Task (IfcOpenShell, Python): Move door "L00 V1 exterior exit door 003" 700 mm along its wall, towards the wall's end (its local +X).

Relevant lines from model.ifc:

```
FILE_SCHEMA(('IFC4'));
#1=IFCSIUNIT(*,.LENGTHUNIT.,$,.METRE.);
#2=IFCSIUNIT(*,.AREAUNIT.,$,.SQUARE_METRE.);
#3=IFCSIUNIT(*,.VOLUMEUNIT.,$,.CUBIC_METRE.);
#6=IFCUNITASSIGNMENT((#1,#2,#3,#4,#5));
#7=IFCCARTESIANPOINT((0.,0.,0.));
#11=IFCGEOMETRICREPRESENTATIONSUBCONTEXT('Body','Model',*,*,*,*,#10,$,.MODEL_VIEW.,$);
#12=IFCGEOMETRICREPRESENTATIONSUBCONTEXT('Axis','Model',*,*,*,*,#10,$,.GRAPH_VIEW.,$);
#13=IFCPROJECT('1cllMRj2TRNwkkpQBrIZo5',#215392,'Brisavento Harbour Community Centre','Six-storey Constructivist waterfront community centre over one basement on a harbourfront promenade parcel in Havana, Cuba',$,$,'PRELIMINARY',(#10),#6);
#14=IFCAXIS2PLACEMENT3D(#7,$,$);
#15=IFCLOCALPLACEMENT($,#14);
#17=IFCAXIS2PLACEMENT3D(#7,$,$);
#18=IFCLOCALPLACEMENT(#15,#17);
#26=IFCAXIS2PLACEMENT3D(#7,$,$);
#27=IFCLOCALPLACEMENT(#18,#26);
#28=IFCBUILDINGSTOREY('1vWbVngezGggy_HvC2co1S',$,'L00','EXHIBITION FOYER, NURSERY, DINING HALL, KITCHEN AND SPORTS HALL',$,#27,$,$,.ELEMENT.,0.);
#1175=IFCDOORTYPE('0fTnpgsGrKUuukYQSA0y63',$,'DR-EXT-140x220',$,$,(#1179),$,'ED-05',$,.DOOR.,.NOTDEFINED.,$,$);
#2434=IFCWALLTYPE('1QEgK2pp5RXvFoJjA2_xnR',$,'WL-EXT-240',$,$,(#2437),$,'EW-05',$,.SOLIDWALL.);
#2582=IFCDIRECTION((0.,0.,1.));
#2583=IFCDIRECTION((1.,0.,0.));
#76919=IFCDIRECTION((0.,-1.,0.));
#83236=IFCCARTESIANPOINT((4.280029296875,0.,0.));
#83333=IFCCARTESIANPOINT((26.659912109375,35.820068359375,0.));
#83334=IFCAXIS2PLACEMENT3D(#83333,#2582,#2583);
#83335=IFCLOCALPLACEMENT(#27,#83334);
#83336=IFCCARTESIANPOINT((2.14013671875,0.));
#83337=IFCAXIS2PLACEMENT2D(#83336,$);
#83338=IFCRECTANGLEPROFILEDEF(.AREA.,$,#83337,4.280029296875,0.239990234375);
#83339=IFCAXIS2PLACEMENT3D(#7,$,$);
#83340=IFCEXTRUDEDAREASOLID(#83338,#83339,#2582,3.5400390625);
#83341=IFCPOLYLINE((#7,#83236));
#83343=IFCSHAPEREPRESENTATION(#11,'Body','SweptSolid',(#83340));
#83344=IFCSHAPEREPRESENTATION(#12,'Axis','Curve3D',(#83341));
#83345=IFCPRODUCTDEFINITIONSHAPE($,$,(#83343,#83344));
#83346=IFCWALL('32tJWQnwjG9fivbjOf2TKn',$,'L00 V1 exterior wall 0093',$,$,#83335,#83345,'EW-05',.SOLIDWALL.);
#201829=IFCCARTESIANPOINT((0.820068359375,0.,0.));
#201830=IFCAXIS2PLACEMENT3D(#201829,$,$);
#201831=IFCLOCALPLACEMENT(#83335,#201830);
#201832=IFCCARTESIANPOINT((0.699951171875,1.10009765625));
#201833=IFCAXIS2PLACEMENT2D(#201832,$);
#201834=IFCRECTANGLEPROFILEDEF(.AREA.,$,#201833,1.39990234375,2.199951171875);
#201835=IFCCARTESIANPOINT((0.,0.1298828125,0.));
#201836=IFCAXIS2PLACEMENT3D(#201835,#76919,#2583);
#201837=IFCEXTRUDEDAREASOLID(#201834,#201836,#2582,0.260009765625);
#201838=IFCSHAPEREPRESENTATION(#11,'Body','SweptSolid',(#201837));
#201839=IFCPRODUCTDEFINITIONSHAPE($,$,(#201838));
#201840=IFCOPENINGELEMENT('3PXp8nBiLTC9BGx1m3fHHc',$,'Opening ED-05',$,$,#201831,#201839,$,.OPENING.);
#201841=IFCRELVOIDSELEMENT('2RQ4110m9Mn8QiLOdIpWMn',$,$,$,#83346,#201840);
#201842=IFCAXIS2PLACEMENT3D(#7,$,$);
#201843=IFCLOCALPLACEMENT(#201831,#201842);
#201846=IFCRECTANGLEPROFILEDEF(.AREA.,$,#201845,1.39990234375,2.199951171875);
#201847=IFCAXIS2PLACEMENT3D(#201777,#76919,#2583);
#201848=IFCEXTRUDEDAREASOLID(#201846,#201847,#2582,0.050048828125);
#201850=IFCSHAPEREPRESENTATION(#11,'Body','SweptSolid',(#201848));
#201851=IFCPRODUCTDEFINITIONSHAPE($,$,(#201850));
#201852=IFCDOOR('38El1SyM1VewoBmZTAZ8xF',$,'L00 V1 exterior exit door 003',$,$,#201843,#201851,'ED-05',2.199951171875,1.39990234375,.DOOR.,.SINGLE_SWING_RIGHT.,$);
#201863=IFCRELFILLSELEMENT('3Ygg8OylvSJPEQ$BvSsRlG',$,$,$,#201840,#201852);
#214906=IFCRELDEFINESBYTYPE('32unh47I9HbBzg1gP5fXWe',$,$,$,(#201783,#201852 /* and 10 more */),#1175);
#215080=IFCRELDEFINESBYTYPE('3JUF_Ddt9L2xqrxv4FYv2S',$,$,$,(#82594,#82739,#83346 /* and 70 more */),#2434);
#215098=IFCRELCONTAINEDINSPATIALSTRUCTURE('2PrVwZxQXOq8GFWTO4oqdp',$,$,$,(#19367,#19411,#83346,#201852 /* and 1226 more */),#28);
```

```python
import ifcopenshell
import ifcopenshell.api.geometry
import ifcopenshell.util.placement
import ifcopenshell.util.unit

model = ifcopenshell.open("model.ifc")
unit_scale = ifcopenshell.util.unit.calculate_unit_scale(model)

door = model.by_guid("38El1SyM1VewoBmZTAZ8xF")
opening = door.FillsVoids[0].RelatingOpeningElement
wall = opening.VoidsElements[0].RelatingBuildingElement

wall_matrix = ifcopenshell.util.placement.get_local_placement(wall.ObjectPlacement)
shift = wall_matrix[:3, 0] * 0.7 / unit_scale
before = ifcopenshell.util.placement.get_local_placement(door.ObjectPlacement)[:3, 3].copy()

# The door is placed relative to its opening, so it follows when the opening moves.
matrix = ifcopenshell.util.placement.get_local_placement(opening.ObjectPlacement)
matrix[:3, 3] += shift
ifcopenshell.api.geometry.edit_object_placement(
    model, product=opening, matrix=matrix, is_si=False, should_transform_children=True
)

after = ifcopenshell.util.placement.get_local_placement(door.ObjectPlacement)[:3, 3]
print("door moved by", (after - before).round(3) + 0.0)

model.write("model_rev.ifc")
```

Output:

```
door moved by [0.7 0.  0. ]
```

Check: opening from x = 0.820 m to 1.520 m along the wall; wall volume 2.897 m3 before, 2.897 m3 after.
